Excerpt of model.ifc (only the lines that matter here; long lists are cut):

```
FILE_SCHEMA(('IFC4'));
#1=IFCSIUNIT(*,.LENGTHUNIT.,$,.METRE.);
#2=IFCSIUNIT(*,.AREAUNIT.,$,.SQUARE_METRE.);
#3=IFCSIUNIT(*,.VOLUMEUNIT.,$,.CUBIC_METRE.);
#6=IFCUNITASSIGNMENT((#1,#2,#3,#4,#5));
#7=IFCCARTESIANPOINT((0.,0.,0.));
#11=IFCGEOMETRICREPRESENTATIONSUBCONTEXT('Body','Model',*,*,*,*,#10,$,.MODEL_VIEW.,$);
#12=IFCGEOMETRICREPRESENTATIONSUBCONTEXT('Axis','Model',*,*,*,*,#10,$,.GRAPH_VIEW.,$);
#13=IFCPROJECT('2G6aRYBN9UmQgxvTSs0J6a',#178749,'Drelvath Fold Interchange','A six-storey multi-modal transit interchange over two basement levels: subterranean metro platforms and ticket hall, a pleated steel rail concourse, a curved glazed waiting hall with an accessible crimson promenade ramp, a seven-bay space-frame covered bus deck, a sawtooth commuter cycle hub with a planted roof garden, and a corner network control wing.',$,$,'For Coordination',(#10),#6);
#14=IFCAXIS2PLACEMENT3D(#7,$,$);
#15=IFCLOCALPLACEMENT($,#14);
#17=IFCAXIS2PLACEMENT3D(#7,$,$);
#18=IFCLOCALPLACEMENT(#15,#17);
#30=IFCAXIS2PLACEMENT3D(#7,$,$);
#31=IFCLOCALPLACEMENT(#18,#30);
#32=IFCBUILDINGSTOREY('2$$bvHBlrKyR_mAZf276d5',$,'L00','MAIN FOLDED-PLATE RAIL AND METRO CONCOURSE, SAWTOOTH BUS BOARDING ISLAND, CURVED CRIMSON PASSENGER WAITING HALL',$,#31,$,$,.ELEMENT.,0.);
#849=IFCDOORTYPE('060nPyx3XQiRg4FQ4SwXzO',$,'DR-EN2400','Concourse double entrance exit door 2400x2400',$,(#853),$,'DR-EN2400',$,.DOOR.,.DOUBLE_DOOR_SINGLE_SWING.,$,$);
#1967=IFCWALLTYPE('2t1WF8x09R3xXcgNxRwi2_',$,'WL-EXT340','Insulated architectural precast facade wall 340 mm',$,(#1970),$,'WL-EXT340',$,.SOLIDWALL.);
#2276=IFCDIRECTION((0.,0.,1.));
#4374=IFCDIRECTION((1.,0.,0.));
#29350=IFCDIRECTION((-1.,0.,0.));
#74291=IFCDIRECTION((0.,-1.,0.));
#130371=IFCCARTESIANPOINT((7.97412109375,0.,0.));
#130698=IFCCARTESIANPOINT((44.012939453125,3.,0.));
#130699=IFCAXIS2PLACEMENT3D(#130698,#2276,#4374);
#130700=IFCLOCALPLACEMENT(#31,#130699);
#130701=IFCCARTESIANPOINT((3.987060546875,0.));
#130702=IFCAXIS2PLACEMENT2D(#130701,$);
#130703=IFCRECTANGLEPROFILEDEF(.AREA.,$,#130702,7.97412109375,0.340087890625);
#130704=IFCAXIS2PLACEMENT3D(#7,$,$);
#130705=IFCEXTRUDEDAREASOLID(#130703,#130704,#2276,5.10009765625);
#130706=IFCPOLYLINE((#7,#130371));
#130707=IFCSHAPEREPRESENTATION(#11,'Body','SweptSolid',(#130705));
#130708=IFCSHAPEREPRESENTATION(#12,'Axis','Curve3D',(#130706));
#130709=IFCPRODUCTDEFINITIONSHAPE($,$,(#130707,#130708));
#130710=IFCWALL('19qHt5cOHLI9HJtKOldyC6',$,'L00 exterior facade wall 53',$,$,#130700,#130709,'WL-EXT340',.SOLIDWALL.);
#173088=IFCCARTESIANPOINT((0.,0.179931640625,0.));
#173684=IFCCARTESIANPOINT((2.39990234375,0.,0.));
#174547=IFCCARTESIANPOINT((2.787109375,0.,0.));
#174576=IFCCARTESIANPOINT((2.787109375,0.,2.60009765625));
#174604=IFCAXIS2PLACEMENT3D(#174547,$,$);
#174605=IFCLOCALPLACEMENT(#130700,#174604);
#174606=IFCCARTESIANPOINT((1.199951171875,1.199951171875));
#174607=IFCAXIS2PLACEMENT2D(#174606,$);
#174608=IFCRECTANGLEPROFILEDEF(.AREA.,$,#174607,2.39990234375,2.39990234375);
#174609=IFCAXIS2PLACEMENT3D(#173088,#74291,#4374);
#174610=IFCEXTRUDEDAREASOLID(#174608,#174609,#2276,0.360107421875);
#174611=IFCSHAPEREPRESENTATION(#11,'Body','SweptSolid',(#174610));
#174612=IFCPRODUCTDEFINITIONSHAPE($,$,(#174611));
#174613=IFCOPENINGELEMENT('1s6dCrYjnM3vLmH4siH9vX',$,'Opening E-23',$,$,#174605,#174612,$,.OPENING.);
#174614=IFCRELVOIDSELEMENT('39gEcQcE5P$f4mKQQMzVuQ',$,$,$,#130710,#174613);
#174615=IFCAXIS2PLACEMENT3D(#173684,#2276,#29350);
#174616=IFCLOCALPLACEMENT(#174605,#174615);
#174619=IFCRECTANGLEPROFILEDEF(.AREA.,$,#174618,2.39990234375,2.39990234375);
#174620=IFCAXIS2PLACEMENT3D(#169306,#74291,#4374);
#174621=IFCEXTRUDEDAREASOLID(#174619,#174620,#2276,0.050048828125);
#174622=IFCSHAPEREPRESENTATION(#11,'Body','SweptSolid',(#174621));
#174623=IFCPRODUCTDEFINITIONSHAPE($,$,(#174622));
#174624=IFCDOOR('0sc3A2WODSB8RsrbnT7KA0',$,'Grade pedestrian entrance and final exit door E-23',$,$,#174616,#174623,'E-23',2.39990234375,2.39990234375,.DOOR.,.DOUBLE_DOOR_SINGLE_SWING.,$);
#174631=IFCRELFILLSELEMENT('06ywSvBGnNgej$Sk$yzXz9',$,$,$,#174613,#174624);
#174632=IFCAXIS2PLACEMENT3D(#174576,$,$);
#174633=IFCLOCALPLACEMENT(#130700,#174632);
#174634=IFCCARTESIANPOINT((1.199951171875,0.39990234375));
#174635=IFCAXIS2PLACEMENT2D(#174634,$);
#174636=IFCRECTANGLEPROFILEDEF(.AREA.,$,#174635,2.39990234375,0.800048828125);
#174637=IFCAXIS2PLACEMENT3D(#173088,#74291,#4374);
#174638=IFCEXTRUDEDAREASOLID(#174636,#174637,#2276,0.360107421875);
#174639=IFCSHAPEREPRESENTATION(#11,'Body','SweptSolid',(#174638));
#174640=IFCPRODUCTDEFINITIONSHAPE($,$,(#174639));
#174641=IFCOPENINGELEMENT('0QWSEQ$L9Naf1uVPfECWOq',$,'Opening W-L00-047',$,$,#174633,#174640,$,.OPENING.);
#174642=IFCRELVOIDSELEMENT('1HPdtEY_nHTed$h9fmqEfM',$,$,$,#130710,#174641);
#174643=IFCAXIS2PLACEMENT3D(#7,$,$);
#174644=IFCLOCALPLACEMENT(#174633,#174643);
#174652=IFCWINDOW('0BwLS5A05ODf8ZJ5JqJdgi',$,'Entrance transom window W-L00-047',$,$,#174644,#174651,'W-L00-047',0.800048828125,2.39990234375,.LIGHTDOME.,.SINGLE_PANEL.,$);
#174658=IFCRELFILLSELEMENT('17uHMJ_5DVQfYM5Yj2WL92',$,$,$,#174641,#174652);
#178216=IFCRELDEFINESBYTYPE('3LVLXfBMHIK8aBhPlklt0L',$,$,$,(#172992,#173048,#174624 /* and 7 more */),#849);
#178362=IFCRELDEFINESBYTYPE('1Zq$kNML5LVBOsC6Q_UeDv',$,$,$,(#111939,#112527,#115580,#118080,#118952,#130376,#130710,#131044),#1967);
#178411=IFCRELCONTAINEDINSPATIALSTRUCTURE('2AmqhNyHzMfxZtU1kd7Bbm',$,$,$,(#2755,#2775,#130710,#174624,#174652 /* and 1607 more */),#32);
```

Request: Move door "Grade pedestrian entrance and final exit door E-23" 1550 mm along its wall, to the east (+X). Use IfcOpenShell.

```python
import ifcopenshell
import ifcopenshell.api.geometry
import ifcopenshell.util.placement
import ifcopenshell.util.unit

model = ifcopenshell.open("model.ifc")
unit_scale = ifcopenshell.util.unit.calculate_unit_scale(model)

door = model.by_id(174624)
opening = door.FillsVoids[0].RelatingOpeningElement
wall = opening.VoidsElements[0].RelatingBuildingElement

wall_matrix = ifcopenshell.util.placement.get_local_placement(wall.ObjectPlacement)
shift = wall_matrix[:3, 0] * 1.55 / unit_scale
before = ifcopenshell.util.placement.get_local_placement(door.ObjectPlacement)[:3, 3].copy()

# The door is placed relative to its opening, so it follows when the opening moves.
matrix = ifcopenshell.util.placement.get_local_placement(opening.ObjectPlacement)
matrix[:3, 3] += shift
ifcopenshell.api.geometry.edit_object_placement(
    model, product=opening, matrix=matrix, is_si=False, should_transform_children=True
)

after = ifcopenshell.util.placement.get_local_placement(door.ObjectPlacement)[:3, 3]
print("door moved by", (after - before).round(3) + 0.0)

model.write("model_v2.ifc")
```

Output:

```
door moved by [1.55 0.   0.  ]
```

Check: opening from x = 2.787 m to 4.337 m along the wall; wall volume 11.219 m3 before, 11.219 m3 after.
